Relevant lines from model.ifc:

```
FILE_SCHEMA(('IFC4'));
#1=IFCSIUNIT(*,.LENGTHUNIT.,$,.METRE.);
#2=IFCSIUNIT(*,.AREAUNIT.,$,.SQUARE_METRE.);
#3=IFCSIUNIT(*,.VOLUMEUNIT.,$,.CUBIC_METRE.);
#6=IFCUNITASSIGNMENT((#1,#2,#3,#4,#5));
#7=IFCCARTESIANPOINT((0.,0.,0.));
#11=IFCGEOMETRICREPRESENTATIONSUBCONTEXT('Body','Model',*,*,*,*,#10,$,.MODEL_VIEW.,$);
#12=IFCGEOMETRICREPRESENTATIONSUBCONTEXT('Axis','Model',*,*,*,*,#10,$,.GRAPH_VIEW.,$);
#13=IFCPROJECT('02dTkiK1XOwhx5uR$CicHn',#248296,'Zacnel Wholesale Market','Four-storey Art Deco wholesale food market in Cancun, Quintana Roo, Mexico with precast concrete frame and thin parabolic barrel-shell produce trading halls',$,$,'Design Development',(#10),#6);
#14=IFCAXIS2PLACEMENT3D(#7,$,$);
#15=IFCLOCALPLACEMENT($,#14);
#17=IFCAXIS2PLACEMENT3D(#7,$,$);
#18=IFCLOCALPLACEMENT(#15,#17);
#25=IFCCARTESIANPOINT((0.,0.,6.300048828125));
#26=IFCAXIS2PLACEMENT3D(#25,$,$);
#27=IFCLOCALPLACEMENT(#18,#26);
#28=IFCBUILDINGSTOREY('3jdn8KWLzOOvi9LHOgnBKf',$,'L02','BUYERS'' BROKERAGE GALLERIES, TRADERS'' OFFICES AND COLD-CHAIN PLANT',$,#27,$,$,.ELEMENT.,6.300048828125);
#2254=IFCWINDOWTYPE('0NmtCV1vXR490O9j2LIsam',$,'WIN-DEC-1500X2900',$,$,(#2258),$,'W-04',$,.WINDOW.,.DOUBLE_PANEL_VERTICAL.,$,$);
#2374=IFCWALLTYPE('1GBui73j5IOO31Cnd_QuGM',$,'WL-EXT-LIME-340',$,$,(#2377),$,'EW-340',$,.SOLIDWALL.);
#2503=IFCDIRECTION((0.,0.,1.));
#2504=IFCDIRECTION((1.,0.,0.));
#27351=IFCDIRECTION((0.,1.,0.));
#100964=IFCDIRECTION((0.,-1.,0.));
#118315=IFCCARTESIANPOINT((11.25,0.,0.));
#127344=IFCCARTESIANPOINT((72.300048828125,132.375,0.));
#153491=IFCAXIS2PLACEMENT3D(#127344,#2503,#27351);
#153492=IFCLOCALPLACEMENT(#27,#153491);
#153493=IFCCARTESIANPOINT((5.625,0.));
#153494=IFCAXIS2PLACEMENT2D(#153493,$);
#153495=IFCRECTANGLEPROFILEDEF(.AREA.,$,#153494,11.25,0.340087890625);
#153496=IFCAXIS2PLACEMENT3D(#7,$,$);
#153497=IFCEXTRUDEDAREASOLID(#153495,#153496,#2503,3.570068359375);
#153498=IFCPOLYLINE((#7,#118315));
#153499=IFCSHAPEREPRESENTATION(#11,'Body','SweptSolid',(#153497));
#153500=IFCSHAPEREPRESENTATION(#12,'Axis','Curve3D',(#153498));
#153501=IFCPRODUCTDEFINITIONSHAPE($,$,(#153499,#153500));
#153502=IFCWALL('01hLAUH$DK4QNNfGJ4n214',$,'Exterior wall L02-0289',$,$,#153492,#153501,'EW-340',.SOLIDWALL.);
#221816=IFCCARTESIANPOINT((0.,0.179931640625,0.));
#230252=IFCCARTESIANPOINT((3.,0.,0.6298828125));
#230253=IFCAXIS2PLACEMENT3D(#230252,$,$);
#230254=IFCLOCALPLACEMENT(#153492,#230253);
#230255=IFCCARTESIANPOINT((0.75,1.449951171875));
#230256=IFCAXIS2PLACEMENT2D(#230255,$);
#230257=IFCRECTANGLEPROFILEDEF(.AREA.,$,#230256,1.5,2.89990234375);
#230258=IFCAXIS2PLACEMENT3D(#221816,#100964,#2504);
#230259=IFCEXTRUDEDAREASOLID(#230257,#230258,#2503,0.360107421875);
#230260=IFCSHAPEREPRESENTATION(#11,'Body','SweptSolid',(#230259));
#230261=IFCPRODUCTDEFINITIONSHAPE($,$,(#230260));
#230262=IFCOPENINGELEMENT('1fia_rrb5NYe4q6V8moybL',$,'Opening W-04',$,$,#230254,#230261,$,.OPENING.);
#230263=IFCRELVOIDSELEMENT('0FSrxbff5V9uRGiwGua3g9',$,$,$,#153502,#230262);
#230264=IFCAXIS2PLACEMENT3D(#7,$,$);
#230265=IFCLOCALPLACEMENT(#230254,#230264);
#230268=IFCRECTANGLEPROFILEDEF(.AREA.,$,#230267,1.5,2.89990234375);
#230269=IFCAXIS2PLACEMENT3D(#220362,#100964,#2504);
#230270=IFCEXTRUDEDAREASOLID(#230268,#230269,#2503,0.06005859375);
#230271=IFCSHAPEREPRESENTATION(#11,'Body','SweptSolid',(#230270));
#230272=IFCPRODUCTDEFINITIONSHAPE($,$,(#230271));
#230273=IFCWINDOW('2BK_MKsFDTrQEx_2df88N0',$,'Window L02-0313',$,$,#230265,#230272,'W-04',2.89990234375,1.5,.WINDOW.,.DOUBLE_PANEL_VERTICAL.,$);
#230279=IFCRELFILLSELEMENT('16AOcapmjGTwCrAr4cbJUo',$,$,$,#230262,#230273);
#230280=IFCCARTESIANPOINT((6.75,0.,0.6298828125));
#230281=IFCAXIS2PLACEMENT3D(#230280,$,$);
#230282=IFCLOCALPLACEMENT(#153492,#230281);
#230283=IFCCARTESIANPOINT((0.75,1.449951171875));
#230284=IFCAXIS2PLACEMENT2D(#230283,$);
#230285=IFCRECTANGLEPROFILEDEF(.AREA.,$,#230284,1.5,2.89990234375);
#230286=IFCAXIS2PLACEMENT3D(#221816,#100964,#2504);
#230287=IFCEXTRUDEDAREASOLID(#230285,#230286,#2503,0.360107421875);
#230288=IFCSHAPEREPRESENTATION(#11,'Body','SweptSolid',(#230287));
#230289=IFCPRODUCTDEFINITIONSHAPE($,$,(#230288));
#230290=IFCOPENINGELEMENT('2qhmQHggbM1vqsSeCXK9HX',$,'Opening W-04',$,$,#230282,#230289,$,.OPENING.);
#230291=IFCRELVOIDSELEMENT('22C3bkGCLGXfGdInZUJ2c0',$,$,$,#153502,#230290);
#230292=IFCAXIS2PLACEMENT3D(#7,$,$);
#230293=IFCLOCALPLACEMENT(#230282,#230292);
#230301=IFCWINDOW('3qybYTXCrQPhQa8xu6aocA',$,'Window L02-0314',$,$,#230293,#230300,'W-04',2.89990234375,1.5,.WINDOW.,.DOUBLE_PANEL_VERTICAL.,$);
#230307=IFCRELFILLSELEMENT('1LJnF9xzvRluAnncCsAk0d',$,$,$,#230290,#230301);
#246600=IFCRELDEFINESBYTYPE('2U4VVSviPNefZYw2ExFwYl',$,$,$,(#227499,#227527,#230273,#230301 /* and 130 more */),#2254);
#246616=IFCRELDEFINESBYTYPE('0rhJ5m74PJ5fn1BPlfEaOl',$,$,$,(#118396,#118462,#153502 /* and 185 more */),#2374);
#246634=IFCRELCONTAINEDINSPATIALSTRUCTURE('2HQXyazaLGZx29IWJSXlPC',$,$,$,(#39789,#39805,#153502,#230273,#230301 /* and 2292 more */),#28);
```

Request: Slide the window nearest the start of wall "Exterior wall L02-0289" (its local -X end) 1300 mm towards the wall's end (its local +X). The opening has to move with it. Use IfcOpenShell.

```python
import ifcopenshell
import ifcopenshell.api.geometry
import ifcopenshell.util.placement

model = ifcopenshell.open("model.ifc")

window = model.by_guid("2BK_MKsFDTrQEx_2df88N0")
opening = window.FillsVoids[0].RelatingOpeningElement
wall = opening.VoidsElements[0].RelatingBuildingElement

wall_matrix = ifcopenshell.util.placement.get_local_placement(wall.ObjectPlacement)
shift = wall_matrix[:3, 0] * 1.3
before = ifcopenshell.util.placement.get_local_placement(window.ObjectPlacement)[:3, 3].copy()

# The window is placed relative to its opening, so it follows when the opening moves.
matrix = ifcopenshell.util.placement.get_local_placement(opening.ObjectPlacement)
matrix[:3, 3] += shift
ifcopenshell.api.geometry.edit_object_placement(
    model, product=opening, matrix=matrix, is_si=False, should_transform_children=True
)

after = ifcopenshell.util.placement.get_local_placement(window.ObjectPlacement)[:3, 3]
print("window moved by", (after - before).round(3) + 0.0)

model.write("model_updated.ifc")
```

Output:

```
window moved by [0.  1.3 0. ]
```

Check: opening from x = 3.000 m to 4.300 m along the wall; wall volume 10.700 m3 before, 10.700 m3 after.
